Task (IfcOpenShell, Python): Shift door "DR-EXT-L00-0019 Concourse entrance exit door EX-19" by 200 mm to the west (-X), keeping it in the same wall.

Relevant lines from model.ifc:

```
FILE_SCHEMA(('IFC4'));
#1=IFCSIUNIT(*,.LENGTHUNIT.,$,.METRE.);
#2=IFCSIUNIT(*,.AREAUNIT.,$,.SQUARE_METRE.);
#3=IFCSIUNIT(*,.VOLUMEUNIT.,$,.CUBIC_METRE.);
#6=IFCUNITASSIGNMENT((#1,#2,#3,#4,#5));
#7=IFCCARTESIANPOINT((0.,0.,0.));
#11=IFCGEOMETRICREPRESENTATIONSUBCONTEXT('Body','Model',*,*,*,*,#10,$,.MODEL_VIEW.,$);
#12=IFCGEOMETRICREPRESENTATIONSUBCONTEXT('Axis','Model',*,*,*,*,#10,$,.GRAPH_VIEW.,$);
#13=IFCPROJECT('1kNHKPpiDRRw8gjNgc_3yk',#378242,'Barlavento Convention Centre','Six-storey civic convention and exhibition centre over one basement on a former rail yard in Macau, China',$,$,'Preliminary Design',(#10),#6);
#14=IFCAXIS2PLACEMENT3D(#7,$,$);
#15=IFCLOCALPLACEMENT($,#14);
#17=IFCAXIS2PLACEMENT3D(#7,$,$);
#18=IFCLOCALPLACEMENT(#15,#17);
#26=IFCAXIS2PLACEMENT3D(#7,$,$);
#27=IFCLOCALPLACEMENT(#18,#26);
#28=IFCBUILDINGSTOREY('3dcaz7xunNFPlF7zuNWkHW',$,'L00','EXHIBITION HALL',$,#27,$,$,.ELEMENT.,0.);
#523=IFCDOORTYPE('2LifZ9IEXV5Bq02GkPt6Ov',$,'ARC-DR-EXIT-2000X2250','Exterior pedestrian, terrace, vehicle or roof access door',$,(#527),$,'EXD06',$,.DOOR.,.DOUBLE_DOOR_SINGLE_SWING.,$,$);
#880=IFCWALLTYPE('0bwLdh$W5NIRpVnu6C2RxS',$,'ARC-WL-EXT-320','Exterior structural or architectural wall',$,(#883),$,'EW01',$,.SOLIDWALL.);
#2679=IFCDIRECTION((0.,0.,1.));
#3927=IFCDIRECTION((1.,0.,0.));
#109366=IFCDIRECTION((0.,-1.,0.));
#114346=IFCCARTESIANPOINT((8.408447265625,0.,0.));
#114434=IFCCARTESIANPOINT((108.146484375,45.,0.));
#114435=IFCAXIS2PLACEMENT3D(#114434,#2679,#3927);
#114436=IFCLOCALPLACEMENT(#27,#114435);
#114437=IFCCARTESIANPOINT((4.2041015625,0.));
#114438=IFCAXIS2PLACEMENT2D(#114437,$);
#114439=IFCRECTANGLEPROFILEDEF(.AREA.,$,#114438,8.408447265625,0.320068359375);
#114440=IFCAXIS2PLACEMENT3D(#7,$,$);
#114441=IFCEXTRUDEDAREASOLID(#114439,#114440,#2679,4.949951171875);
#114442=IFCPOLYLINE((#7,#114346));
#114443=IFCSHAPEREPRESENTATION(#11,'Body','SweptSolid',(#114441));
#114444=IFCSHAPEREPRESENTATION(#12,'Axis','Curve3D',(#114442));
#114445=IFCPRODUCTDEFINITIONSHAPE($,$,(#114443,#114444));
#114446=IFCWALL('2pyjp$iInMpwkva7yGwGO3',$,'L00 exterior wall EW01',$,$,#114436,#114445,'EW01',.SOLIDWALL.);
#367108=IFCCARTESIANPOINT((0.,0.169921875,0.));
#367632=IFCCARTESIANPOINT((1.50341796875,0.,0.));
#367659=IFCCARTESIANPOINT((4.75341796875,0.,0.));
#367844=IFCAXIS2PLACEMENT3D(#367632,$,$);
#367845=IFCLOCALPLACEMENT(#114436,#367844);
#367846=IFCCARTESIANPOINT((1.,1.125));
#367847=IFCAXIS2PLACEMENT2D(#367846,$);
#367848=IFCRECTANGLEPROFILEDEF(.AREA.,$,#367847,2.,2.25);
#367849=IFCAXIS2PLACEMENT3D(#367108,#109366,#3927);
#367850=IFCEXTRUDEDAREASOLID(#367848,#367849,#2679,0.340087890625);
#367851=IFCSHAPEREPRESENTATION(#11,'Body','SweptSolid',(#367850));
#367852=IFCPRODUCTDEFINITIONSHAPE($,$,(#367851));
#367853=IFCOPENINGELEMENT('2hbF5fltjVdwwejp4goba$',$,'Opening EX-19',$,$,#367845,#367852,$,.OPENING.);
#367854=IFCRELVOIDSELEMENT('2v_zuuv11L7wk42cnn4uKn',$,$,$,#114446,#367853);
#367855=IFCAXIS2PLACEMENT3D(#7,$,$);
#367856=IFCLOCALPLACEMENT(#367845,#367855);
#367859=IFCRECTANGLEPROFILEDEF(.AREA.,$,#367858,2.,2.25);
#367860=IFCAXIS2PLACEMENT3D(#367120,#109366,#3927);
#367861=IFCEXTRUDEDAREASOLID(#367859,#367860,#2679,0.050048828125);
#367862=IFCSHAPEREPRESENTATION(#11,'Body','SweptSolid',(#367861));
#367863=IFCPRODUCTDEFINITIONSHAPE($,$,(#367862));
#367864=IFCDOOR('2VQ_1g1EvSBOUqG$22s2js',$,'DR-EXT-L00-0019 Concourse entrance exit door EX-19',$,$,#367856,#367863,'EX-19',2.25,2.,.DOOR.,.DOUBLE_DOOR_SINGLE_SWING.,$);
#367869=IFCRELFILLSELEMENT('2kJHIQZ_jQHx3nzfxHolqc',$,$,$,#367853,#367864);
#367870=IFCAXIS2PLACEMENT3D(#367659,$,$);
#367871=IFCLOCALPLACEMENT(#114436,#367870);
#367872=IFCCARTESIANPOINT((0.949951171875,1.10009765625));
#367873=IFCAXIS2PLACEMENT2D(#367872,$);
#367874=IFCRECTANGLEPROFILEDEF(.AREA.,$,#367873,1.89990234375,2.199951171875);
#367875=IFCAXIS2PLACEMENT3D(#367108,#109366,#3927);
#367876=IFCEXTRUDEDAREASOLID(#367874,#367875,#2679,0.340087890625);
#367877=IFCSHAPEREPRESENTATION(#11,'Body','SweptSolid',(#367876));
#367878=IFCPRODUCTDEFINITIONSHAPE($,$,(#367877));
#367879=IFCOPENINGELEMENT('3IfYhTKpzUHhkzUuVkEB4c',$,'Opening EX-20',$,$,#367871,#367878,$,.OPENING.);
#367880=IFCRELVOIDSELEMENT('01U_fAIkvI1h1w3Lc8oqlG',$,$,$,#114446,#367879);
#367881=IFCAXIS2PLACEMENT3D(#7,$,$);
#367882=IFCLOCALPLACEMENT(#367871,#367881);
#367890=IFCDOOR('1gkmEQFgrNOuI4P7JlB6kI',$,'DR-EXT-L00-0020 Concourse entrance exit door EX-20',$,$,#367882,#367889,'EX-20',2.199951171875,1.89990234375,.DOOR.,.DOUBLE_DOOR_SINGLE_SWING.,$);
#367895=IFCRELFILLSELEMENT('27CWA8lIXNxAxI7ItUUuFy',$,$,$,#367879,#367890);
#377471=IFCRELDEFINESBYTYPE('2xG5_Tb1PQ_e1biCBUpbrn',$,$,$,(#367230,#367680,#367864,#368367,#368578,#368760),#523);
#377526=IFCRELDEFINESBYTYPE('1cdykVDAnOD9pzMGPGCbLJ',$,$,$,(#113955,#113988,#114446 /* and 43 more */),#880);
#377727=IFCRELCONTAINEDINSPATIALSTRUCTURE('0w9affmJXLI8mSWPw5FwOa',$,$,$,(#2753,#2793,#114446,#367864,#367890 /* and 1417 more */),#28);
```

```python
import ifcopenshell
import ifcopenshell.api.geometry
import ifcopenshell.util.placement

model = ifcopenshell.open("model.ifc")

door = model.by_id(367864)
opening = door.FillsVoids[0].RelatingOpeningElement
wall = opening.VoidsElements[0].RelatingBuildingElement

wall_matrix = ifcopenshell.util.placement.get_local_placement(wall.ObjectPlacement)
shift = wall_matrix[:3, 0] * -0.2
before = ifcopenshell.util.placement.get_local_placement(door.ObjectPlacement)[:3, 3].copy()

# The door is placed relative to its opening, so it follows when the opening moves.
matrix = ifcopenshell.util.placement.get_local_placement(opening.ObjectPlacement)
matrix[:3, 3] += shift
ifcopenshell.api.geometry.edit_object_placement(
    model, product=opening, matrix=matrix, is_si=False, should_transform_children=True
)

after = ifcopenshell.util.placement.get_local_placement(door.ObjectPlacement)[:3, 3]
print("door moved by", (after - before).round(3) + 0.0)

model.write("model_rev.ifc")
```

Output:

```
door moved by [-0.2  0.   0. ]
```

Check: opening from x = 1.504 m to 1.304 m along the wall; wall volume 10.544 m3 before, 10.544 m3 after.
